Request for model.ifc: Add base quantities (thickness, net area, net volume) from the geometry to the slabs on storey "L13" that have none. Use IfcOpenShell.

First a look at what the model holds.

```python
import ifcopenshell
import ifcopenshell.util.element
import ifcopenshell.util.unit

model = ifcopenshell.open("model.ifc")
print(model.schema)
for unit_type in ("LENGTHUNIT", "AREAUNIT", "VOLUMEUNIT"):
    print(unit_type, ifcopenshell.util.unit.calculate_unit_scale(model, unit_type))
storey = next(s for s in model.by_type("IfcBuildingStorey") if s.Name == "L13")
slabs = [e for e in ifcopenshell.util.element.get_decomposition(storey) if e.is_a("IfcSlab")]
for e in sorted(slabs, key=lambda e: e.id()):
    print(e.id(), e.is_a(), e.Name, list(ifcopenshell.util.element.get_psets(e, qtos_only=True)), sep=" | ")
```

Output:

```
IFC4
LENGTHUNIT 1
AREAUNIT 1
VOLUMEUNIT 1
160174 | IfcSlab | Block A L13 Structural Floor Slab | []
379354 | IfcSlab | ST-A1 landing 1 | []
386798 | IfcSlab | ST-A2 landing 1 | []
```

```python
import ifcopenshell
import ifcopenshell.api.pset
import ifcopenshell.geom
import ifcopenshell.util.element
import ifcopenshell.util.shape
import ifcopenshell.util.unit

model = ifcopenshell.open("model.ifc")
unit_scale = ifcopenshell.util.unit.calculate_unit_scale(model)
area_scale = ifcopenshell.util.unit.calculate_unit_scale(model, "AREAUNIT")
volume_scale = ifcopenshell.util.unit.calculate_unit_scale(model, "VOLUMEUNIT")
settings = ifcopenshell.geom.settings()

storey = next(s for s in model.by_type("IfcBuildingStorey") if s.Name == "L13")
slabs = [e for e in ifcopenshell.util.element.get_decomposition(storey) if e.is_a("IfcSlab")]

for e in sorted(slabs, key=lambda e: e.id()):
    if ifcopenshell.util.element.get_psets(e, qtos_only=True, should_inherit=False):
        continue
    # Geometry comes back in metres, in the element's own axes.
    shape = ifcopenshell.geom.create_shape(settings, e)
    values = {
        "Width": ifcopenshell.util.shape.get_z(shape.geometry) / unit_scale,
        "NetArea": ifcopenshell.util.shape.get_footprint_area(shape.geometry) / area_scale,
        "NetVolume": ifcopenshell.util.shape.get_volume(shape.geometry) / volume_scale,
    }
    qto = ifcopenshell.api.pset.add_qto(model, product=e, name="Qto_SlabBaseQuantities")
    ifcopenshell.api.pset.edit_qto(model, qto=qto, properties=values)
    print(e.id(), {k: round(v, 3) for k, v in values.items()})

model.write("model_v2.ifc")
```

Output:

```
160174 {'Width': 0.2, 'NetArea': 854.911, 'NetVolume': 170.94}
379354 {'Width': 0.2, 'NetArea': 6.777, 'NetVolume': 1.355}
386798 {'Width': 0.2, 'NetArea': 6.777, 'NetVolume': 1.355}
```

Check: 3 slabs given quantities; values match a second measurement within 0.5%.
